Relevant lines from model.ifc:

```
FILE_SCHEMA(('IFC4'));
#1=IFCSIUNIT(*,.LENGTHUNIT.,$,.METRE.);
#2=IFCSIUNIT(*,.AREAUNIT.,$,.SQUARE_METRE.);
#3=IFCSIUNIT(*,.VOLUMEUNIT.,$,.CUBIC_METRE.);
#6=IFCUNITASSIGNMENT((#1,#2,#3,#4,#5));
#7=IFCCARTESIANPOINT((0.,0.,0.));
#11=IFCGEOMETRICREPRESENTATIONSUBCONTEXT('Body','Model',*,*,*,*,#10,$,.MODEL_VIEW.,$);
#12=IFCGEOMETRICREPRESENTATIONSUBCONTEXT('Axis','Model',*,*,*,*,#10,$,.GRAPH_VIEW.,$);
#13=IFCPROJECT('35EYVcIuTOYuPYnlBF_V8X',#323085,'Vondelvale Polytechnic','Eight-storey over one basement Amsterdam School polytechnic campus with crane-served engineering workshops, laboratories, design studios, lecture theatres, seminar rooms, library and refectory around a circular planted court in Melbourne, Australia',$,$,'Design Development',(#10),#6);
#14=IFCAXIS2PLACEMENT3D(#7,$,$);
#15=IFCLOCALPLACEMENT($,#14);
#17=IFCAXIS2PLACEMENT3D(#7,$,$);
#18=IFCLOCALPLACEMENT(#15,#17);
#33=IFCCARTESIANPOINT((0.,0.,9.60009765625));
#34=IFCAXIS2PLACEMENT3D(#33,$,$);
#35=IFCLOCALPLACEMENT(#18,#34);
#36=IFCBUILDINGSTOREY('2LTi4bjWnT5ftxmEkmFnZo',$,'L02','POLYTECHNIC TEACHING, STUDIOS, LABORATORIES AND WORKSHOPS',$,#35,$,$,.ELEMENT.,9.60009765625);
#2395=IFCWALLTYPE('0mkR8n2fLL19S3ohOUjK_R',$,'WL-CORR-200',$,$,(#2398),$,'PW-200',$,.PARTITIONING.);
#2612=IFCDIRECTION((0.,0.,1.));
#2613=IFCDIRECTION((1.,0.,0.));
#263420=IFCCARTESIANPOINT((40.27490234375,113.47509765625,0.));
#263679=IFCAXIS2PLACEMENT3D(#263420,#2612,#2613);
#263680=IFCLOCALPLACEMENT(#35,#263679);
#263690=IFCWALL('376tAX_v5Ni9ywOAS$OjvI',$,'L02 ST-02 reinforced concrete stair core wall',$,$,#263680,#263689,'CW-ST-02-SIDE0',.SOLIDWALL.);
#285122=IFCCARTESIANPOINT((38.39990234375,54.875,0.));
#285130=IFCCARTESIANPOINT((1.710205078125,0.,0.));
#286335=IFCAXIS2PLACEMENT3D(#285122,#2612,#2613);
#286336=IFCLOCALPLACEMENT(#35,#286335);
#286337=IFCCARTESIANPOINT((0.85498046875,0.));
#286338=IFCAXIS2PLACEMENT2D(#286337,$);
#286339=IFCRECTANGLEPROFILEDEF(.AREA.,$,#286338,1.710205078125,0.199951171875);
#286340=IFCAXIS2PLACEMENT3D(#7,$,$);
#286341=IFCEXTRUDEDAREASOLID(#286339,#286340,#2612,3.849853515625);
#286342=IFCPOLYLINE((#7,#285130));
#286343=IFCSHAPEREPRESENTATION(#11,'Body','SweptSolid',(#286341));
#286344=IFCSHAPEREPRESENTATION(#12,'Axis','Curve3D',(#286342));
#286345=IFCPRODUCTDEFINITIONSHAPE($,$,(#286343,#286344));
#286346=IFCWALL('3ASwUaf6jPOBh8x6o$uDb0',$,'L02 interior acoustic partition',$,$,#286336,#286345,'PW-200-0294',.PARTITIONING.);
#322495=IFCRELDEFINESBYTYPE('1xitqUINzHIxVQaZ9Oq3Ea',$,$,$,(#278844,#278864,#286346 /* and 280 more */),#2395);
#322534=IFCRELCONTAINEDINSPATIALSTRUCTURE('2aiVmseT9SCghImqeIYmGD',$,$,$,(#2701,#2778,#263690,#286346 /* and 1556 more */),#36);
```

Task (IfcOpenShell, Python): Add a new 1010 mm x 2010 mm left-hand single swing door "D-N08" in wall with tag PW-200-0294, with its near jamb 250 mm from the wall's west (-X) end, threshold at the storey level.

```python
import numpy as np
import ifcopenshell
import ifcopenshell.api.feature
import ifcopenshell.api.geometry
import ifcopenshell.api.root
import ifcopenshell.api.spatial
import ifcopenshell.geom
import ifcopenshell.util.element
import ifcopenshell.util.placement
import ifcopenshell.util.representation
import ifcopenshell.util.shape
import ifcopenshell.util.unit

model = ifcopenshell.open("model.ifc")
unit_scale = ifcopenshell.util.unit.calculate_unit_scale(model)
settings = ifcopenshell.geom.settings()


def volume(element):
    """Net volume in cubic metres, openings subtracted."""
    shape = ifcopenshell.geom.create_shape(settings, element)
    return ifcopenshell.util.shape.get_volume(shape.geometry)


wall = model.by_guid("3ASwUaf6jPOBh8x6o$uDb0")
storey = ifcopenshell.util.element.get_container(wall, ifc_class="IfcBuildingStorey")
context = ifcopenshell.util.representation.get_context(model, "Model", "Body", "MODEL_VIEW")
before = volume(wall)

width, height, from_end, sill = 1.01, 2.01, 0.25, 0.0  # metres

# The wall runs along its own X axis, and the end named is its -X end.
wall_shape = ifcopenshell.geom.create_shape(settings, wall)
x, y, z = ifcopenshell.util.shape.get_vertices(wall_shape.geometry).T
start = x.min() + from_end
face, thickness = float(y.min()), float(y.max() - y.min())
wall_matrix = ifcopenshell.util.placement.get_local_placement(wall.ObjectPlacement)
level = ifcopenshell.util.placement.get_local_placement(storey.ObjectPlacement)[2, 3]


def in_wall(x, y):
    """Placement at x, y metres in the wall's axes, at sill height."""
    matrix = wall_matrix.copy()
    matrix[:, 3] = wall_matrix @ np.array([x / unit_scale, y / unit_scale, 0.0, 1.0])
    matrix[2, 3] = level + sill / unit_scale
    return matrix


# Opening: a box that overshoots both wall faces by 50 mm.
opening = ifcopenshell.api.root.create_entity(model, ifc_class="IfcOpeningElement", predefined_type="OPENING")
box = ifcopenshell.api.geometry.add_wall_representation(
    model, context=context, length=width, height=height, thickness=thickness + 0.1
)
ifcopenshell.api.geometry.assign_representation(model, product=opening, representation=box)
ifcopenshell.api.geometry.edit_object_placement(model, product=opening, matrix=in_wall(start, face - 0.05), is_si=False)
ifcopenshell.api.feature.add_feature(model, feature=opening, element=wall)

door = ifcopenshell.api.root.create_entity(model, ifc_class="IfcDoor", name="D-N08", predefined_type="DOOR")
door.OverallWidth, door.OverallHeight = width / unit_scale, height / unit_scale
door.OperationType = "SINGLE_SWING_LEFT"
body = ifcopenshell.api.geometry.add_door_representation(
    model,
    context=context,
    overall_width=door.OverallWidth,
    overall_height=door.OverallHeight,
    operation_type="SINGLE_SWING_LEFT",
    lining_properties={"LiningDepth": thickness / unit_scale, "ThresholdDepth": thickness / unit_scale},
)
ifcopenshell.api.geometry.assign_representation(model, product=door, representation=body)
ifcopenshell.api.spatial.assign_container(model, products=[door], relating_structure=storey)
ifcopenshell.api.feature.add_filling(model, opening=opening, element=door)

# The lining spans the wall, so the door starts at the wall face.
ifcopenshell.api.geometry.edit_object_placement(model, product=door, matrix=in_wall(start, face), is_si=False)

after = volume(wall)

print(f"wall volume {before:.3f} -> {after:.3f} m3")

model.write("model_updated.ifc")
```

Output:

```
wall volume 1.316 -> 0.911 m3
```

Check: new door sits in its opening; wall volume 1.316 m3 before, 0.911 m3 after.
